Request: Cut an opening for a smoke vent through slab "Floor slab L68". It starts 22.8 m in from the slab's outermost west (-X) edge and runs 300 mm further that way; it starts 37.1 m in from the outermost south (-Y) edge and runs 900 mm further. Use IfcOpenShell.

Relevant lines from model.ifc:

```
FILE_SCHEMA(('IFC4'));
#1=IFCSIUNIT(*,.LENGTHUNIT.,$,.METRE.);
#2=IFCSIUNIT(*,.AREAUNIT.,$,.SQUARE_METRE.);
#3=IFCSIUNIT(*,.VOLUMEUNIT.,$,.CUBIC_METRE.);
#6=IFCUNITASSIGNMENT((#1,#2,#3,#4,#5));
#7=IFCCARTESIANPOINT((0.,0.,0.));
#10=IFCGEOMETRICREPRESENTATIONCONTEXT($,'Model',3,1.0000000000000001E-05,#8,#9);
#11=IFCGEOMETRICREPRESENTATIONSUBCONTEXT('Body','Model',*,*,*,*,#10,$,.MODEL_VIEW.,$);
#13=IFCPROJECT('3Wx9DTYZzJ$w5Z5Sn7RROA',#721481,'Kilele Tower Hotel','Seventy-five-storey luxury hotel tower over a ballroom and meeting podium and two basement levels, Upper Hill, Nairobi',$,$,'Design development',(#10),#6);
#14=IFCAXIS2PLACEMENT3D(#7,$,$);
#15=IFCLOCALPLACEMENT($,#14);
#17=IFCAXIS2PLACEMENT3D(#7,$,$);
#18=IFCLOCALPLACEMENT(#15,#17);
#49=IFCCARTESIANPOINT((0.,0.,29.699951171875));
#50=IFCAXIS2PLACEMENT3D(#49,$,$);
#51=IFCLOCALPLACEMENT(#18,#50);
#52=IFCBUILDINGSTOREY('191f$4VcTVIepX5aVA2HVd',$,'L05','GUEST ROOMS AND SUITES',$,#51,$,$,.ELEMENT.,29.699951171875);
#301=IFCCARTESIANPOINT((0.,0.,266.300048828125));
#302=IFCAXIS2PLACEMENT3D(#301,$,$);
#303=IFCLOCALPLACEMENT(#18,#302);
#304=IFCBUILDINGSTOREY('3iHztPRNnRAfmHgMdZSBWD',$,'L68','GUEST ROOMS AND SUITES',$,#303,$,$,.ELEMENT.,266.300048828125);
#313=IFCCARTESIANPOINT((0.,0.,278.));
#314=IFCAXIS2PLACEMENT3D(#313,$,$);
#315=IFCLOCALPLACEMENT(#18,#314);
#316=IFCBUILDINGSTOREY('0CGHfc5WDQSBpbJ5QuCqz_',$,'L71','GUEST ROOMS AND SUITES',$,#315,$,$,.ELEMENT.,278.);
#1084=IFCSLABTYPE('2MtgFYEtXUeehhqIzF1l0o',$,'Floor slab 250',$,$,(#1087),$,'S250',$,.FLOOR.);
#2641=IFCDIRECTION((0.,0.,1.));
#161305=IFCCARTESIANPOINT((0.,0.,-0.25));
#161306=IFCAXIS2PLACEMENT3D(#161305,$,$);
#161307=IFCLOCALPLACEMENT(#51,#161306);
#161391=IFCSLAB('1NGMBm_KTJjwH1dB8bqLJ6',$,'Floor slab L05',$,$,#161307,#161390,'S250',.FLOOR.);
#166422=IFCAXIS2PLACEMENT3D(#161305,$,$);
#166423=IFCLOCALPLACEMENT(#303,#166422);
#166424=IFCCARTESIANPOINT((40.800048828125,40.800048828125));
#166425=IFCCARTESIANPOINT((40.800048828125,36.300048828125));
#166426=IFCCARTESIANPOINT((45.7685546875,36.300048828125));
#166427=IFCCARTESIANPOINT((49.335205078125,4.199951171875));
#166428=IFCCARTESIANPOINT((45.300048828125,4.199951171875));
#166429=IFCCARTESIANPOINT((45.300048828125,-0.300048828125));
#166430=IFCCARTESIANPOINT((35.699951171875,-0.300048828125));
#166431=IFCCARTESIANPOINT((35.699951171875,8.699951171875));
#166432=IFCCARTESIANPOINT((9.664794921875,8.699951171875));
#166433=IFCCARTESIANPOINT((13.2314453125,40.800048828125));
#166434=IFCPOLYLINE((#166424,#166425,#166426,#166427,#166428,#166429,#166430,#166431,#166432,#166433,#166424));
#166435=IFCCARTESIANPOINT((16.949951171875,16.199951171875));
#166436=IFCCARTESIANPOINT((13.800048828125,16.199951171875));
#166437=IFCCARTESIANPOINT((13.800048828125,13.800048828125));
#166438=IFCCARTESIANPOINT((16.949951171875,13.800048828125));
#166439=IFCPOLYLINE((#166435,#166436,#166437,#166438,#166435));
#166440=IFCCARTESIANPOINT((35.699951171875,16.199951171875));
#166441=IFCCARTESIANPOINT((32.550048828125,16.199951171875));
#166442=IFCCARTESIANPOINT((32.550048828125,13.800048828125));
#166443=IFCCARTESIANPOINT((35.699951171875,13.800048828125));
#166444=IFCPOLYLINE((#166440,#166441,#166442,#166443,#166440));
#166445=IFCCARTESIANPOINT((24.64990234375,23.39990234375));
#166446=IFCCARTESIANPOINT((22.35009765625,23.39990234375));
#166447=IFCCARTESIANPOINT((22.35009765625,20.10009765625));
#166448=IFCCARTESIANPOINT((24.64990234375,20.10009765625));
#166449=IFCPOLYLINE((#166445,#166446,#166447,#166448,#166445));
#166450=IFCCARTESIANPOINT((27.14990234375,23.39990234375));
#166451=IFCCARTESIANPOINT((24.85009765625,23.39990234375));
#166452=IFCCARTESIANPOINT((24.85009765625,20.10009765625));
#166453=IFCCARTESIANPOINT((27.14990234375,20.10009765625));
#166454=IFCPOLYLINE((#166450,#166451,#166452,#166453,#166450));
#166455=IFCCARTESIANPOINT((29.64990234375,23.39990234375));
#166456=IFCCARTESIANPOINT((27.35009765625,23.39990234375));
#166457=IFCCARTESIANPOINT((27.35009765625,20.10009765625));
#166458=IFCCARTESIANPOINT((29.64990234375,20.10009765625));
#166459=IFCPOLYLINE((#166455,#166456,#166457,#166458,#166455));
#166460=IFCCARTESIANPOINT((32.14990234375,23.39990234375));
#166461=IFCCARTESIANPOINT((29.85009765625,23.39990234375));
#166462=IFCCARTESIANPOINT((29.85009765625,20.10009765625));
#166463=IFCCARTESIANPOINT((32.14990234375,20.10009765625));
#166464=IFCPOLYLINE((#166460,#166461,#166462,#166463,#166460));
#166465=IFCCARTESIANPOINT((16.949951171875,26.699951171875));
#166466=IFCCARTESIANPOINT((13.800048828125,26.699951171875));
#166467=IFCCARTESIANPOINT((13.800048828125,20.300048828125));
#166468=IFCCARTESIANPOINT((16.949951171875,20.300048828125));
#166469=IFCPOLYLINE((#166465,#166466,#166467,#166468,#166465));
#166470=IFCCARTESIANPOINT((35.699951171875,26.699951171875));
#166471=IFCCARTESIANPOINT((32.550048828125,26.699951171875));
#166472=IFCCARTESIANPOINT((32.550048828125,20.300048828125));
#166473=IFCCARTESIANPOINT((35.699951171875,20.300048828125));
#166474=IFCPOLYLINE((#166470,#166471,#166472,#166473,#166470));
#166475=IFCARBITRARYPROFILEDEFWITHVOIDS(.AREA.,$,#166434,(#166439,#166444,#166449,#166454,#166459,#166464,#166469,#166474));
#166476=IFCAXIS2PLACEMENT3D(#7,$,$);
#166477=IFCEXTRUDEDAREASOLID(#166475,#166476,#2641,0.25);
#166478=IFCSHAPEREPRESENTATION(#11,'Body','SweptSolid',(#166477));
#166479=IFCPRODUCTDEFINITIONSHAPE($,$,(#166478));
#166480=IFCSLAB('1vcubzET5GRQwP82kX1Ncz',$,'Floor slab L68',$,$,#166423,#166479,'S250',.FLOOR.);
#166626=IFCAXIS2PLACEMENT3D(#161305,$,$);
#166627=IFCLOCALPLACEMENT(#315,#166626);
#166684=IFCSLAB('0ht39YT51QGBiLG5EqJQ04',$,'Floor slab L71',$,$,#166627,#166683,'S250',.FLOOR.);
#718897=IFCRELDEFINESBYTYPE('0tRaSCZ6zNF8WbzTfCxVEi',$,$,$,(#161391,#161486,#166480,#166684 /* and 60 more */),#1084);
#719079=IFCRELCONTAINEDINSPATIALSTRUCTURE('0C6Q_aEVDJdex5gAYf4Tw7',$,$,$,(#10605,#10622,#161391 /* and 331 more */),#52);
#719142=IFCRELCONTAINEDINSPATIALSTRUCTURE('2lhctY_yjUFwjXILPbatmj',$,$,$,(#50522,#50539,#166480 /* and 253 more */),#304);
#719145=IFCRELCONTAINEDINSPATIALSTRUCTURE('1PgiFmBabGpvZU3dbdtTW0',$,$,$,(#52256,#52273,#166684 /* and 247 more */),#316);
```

```python
import numpy as np
import ifcopenshell
import ifcopenshell.api.feature
import ifcopenshell.api.geometry
import ifcopenshell.api.root
import ifcopenshell.geom
import ifcopenshell.util.placement
import ifcopenshell.util.representation
import ifcopenshell.util.shape
import ifcopenshell.util.unit

model = ifcopenshell.open("model.ifc")
unit_scale = ifcopenshell.util.unit.calculate_unit_scale(model)
settings = ifcopenshell.geom.settings()


def volume(element):
    """Net volume in cubic metres, openings subtracted."""
    shape = ifcopenshell.geom.create_shape(settings, element)
    return ifcopenshell.util.shape.get_volume(shape.geometry)


slab = model.by_id(166480)
before = volume(slab)

# Extent in the slab's own axes, in metres. The edges named are its -X and -Y sides.
slab_shape = ifcopenshell.geom.create_shape(settings, slab)
vertices = ifcopenshell.util.shape.get_vertices(slab_shape.geometry)
x_min, y_min, bottom = vertices.min(axis=0)
top = vertices[:, 2].max()

opening = ifcopenshell.api.root.create_entity(model, ifc_class="IfcOpeningElement", name="Smoke vent opening", predefined_type="OPENING")
context = ifcopenshell.util.representation.get_context(model, "Model", "Body", "MODEL_VIEW")
width, depth = 0.3, 0.9
outline = [(0.0, 0.0), (width, 0.0), (width, depth), (0.0, depth), (0.0, 0.0)]
# Overshoot both faces by 50 mm so the cut is clean.
shape = ifcopenshell.api.geometry.add_slab_representation(
    model, context=context, depth=top - bottom + 0.1, polyline=outline
)
ifcopenshell.api.geometry.assign_representation(model, product=opening, representation=shape)

matrix = ifcopenshell.util.placement.get_local_placement(slab.ObjectPlacement)
matrix[:, 3] = matrix @ np.append(np.array([x_min + 22.8, y_min + 37.1, bottom - 0.05]) / unit_scale, 1.0)
ifcopenshell.api.geometry.edit_object_placement(model, product=opening, matrix=matrix, is_si=False)
ifcopenshell.api.feature.add_feature(model, feature=opening, element=slab)

after = volume(slab)

print(f"slab volume {before:.3f} -> {after:.3f} m3")

model.write("model_edited.ifc")
```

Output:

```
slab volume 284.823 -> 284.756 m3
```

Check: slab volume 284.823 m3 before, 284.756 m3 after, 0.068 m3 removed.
